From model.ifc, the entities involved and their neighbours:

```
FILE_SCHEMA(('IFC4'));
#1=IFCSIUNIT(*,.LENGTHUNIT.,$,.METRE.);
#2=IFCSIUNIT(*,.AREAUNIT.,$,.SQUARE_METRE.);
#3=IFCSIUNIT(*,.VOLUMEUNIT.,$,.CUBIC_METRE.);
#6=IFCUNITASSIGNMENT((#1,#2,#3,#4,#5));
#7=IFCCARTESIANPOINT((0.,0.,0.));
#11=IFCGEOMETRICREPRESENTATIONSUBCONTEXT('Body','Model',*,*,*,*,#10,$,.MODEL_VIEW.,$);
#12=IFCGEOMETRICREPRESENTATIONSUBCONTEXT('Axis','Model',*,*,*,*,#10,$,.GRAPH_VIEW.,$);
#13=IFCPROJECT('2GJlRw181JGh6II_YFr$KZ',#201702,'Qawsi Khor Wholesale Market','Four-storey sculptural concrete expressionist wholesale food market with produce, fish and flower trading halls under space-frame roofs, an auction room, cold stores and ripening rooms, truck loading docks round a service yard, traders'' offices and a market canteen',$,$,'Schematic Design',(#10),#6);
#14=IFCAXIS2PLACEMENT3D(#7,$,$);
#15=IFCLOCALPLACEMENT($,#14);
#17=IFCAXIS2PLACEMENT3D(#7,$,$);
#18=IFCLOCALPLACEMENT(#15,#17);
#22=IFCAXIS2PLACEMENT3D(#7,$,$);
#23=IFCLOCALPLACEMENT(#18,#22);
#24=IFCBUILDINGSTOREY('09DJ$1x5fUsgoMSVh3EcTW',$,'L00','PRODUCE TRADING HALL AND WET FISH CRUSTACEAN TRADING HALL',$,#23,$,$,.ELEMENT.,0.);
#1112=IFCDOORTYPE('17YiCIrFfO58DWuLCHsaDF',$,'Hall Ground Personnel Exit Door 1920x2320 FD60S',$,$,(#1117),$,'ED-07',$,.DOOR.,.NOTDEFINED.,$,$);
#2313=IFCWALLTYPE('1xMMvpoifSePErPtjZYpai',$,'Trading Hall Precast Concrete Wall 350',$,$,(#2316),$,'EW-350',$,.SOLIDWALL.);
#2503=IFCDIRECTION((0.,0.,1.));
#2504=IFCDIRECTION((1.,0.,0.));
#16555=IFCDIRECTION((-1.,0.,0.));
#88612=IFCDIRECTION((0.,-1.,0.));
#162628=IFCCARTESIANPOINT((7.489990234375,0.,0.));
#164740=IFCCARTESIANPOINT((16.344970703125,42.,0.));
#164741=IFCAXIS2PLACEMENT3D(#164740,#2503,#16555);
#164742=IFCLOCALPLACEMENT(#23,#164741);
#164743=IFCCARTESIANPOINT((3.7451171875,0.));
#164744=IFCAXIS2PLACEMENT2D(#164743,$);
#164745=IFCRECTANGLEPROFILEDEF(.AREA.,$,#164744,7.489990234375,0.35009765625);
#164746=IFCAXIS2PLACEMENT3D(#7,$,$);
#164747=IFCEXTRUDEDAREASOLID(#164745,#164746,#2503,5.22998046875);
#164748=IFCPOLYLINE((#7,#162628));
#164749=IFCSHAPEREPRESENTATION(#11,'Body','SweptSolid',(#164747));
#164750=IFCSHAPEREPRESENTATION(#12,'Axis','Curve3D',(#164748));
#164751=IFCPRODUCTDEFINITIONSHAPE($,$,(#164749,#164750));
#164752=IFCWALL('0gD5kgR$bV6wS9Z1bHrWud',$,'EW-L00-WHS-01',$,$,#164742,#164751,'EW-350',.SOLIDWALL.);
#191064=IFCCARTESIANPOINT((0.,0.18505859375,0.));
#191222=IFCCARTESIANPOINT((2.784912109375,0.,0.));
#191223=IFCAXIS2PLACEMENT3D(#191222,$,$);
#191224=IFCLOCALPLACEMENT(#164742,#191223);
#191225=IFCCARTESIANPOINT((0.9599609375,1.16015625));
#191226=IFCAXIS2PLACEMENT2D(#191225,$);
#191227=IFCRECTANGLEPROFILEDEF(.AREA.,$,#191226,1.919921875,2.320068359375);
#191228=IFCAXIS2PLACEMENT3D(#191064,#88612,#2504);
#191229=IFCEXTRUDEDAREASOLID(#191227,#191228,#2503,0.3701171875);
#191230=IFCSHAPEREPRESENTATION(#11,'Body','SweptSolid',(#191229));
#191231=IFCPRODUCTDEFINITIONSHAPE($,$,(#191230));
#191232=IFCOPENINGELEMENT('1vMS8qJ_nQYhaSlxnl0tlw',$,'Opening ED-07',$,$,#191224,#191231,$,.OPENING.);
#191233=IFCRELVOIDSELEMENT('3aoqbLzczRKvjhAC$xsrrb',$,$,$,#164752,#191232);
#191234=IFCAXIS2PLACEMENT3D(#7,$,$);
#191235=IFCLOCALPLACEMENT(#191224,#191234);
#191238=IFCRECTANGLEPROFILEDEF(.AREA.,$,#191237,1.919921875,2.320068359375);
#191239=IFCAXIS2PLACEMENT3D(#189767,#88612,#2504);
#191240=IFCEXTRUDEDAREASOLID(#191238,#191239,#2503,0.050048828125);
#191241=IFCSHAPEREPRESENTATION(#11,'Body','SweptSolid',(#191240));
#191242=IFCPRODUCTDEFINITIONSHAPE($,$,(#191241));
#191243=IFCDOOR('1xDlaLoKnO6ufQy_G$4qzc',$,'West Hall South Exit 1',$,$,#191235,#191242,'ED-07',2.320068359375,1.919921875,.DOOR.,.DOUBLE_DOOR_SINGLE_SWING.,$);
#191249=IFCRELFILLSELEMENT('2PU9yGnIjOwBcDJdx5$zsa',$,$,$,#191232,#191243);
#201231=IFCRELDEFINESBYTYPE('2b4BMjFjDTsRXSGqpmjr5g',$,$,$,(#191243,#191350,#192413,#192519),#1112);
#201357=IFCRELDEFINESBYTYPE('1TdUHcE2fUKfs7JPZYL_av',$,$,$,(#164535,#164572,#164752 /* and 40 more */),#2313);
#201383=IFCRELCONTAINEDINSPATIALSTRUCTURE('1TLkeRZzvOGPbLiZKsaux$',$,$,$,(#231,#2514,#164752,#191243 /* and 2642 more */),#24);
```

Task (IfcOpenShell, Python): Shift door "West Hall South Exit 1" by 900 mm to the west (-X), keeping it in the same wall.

```python
import ifcopenshell
import ifcopenshell.api.geometry
import ifcopenshell.util.placement
import ifcopenshell.util.unit

model = ifcopenshell.open("model.ifc")
unit_scale = ifcopenshell.util.unit.calculate_unit_scale(model)

door = model.by_guid("1xDlaLoKnO6ufQy_G$4qzc")
opening = door.FillsVoids[0].RelatingOpeningElement
wall = opening.VoidsElements[0].RelatingBuildingElement

wall_matrix = ifcopenshell.util.placement.get_local_placement(wall.ObjectPlacement)
shift = wall_matrix[:3, 0] * 0.9 / unit_scale
before = ifcopenshell.util.placement.get_local_placement(door.ObjectPlacement)[:3, 3].copy()

# The door is placed relative to its opening, so it follows when the opening moves.
matrix = ifcopenshell.util.placement.get_local_placement(opening.ObjectPlacement)
matrix[:3, 3] += shift
ifcopenshell.api.geometry.edit_object_placement(
    model, product=opening, matrix=matrix, is_si=False, should_transform_children=True
)

after = ifcopenshell.util.placement.get_local_placement(door.ObjectPlacement)[:3, 3]
print("door moved by", (after - before).round(3) + 0.0)

model.write("model_v2.ifc")
```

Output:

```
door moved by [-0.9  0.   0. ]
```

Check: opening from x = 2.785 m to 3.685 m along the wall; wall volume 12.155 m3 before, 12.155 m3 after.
